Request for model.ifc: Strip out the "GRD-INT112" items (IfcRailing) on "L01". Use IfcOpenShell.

First a look at what the model holds.

```python
import ifcopenshell
import ifcopenshell.util.element

model = ifcopenshell.open("model.ifc")
print(model.schema)
storey = next(s for s in model.by_type("IfcBuildingStorey") if s.Name == "L01")
railings = [e for e in ifcopenshell.util.element.get_decomposition(storey) if e.is_a("IfcRailing")]
seen = {}
for e in railings:
    element_type = ifcopenshell.util.element.get_type(e)
    name = element_type.Name if element_type not in (None, e) else None
    seen[name] = seen.get(name, 0) + 1
for name, count in sorted(seen.items(), key=str):
    print(count, "x", name)
```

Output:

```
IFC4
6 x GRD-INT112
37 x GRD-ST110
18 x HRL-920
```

```python
import ifcopenshell
import ifcopenshell.api.root
import ifcopenshell.util.element

model = ifcopenshell.open("model.ifc")

storey = next(s for s in model.by_type("IfcBuildingStorey") if s.Name == "L01")
railings = [e for e in ifcopenshell.util.element.get_decomposition(storey) if e.is_a("IfcRailing")]
targets = [e for e in railings if (t := ifcopenshell.util.element.get_type(e)) not in (None, e) and t.Name == "GRD-INT112"]

for e in targets:
    ifcopenshell.api.root.remove_product(model, product=e)
print(len(targets), "removed")

model.write("model-out.ifc")
```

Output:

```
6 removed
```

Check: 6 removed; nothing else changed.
